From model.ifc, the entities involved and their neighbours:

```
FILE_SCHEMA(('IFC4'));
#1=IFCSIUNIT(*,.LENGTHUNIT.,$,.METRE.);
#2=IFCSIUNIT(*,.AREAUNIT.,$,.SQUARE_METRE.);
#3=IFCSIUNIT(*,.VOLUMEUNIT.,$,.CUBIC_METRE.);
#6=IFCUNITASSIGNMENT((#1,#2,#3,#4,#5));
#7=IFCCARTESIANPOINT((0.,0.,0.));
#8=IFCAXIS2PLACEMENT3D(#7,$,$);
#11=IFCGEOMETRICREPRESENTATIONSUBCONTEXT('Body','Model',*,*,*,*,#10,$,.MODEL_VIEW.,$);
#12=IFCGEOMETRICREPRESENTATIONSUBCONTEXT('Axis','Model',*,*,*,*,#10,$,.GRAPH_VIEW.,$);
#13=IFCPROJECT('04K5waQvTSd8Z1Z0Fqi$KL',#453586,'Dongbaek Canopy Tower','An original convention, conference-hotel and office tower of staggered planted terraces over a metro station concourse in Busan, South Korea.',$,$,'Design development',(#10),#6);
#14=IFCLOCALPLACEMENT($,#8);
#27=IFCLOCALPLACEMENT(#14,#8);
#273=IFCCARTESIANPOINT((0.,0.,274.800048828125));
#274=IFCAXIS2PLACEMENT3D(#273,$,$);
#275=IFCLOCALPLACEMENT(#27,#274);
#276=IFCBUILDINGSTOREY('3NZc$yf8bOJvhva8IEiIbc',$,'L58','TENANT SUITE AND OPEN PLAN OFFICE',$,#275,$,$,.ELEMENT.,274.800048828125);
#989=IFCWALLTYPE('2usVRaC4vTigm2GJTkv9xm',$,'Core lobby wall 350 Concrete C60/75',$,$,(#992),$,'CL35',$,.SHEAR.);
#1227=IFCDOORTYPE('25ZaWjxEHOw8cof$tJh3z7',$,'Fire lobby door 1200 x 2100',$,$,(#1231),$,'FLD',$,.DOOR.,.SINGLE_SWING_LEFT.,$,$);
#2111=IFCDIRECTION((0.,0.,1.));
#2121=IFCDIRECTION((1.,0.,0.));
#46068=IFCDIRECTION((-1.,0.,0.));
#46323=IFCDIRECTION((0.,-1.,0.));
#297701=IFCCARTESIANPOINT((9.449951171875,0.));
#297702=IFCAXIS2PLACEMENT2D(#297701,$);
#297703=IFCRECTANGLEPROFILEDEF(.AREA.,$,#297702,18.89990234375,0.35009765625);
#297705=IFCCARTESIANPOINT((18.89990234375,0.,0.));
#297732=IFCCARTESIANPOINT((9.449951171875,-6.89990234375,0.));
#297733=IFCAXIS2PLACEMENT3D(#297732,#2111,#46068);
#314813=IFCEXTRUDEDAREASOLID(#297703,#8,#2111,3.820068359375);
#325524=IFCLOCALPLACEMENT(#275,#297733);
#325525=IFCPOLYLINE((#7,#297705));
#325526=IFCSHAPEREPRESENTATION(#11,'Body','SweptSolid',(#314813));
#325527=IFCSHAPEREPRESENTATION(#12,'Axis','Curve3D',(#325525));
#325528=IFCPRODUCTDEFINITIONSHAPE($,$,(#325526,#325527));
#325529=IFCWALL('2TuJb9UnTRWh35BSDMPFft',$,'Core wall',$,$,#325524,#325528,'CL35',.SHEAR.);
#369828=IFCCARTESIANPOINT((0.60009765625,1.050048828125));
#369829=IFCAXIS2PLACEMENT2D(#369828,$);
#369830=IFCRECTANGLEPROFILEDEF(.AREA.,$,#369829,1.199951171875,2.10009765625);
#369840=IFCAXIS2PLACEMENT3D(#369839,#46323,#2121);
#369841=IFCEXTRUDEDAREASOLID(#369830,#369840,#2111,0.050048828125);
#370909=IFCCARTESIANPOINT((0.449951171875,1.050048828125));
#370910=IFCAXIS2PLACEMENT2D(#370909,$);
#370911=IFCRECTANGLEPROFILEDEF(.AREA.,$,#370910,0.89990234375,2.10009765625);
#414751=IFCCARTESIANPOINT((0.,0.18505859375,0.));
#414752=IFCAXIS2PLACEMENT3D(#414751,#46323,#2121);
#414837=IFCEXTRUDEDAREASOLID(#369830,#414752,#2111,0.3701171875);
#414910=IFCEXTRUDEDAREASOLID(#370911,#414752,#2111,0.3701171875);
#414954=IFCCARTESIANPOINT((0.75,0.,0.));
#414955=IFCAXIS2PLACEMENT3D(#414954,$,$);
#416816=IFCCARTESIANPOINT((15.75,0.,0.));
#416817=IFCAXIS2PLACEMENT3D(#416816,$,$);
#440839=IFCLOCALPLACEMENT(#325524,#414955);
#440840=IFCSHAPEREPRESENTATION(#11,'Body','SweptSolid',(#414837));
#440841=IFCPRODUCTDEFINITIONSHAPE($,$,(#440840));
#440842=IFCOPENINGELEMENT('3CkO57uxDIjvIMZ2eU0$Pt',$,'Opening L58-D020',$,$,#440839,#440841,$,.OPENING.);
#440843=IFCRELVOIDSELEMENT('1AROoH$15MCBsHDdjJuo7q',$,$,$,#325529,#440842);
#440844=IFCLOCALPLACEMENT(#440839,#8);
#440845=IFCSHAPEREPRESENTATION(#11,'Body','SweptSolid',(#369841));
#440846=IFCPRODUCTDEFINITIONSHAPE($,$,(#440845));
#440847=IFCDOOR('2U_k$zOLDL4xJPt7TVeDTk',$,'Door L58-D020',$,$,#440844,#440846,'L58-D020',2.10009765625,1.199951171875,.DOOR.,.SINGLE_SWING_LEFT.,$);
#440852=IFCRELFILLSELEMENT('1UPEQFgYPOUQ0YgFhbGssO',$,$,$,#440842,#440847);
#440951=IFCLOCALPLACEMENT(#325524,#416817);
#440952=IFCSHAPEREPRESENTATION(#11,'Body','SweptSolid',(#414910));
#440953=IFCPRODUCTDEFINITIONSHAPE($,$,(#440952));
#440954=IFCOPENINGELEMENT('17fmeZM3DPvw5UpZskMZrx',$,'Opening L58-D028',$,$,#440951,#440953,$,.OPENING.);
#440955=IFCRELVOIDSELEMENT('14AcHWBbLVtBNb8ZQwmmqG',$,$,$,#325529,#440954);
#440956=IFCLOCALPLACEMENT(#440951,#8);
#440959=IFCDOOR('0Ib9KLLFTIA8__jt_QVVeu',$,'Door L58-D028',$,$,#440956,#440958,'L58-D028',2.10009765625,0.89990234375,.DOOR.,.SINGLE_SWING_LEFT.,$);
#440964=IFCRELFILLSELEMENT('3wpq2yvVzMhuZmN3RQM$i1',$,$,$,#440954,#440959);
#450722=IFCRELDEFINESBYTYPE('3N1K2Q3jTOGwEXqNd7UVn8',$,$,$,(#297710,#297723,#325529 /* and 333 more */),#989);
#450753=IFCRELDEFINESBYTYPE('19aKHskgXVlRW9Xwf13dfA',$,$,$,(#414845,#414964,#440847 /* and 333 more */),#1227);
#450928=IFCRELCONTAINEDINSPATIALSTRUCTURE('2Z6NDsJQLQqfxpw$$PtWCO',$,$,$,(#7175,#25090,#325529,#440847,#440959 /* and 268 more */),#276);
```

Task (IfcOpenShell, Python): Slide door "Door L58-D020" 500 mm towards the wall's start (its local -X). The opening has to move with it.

```python
import ifcopenshell
import ifcopenshell.api.geometry
import ifcopenshell.util.placement

model = ifcopenshell.open("model.ifc")

door = model.by_id(440847)
opening = door.FillsVoids[0].RelatingOpeningElement
wall = opening.VoidsElements[0].RelatingBuildingElement

wall_matrix = ifcopenshell.util.placement.get_local_placement(wall.ObjectPlacement)
shift = wall_matrix[:3, 0] * -0.5
before = ifcopenshell.util.placement.get_local_placement(door.ObjectPlacement)[:3, 3].copy()

# The door is placed relative to its opening, so it follows when the opening moves.
matrix = ifcopenshell.util.placement.get_local_placement(opening.ObjectPlacement)
matrix[:3, 3] += shift
ifcopenshell.api.geometry.edit_object_placement(
    model, product=opening, matrix=matrix, is_si=False, should_transform_children=True
)

after = ifcopenshell.util.placement.get_local_placement(door.ObjectPlacement)[:3, 3]
print("door moved by", (after - before).round(3) + 0.0)

model.write("model_updated.ifc")
```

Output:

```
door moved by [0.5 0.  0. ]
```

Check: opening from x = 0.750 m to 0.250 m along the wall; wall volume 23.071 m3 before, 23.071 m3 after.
